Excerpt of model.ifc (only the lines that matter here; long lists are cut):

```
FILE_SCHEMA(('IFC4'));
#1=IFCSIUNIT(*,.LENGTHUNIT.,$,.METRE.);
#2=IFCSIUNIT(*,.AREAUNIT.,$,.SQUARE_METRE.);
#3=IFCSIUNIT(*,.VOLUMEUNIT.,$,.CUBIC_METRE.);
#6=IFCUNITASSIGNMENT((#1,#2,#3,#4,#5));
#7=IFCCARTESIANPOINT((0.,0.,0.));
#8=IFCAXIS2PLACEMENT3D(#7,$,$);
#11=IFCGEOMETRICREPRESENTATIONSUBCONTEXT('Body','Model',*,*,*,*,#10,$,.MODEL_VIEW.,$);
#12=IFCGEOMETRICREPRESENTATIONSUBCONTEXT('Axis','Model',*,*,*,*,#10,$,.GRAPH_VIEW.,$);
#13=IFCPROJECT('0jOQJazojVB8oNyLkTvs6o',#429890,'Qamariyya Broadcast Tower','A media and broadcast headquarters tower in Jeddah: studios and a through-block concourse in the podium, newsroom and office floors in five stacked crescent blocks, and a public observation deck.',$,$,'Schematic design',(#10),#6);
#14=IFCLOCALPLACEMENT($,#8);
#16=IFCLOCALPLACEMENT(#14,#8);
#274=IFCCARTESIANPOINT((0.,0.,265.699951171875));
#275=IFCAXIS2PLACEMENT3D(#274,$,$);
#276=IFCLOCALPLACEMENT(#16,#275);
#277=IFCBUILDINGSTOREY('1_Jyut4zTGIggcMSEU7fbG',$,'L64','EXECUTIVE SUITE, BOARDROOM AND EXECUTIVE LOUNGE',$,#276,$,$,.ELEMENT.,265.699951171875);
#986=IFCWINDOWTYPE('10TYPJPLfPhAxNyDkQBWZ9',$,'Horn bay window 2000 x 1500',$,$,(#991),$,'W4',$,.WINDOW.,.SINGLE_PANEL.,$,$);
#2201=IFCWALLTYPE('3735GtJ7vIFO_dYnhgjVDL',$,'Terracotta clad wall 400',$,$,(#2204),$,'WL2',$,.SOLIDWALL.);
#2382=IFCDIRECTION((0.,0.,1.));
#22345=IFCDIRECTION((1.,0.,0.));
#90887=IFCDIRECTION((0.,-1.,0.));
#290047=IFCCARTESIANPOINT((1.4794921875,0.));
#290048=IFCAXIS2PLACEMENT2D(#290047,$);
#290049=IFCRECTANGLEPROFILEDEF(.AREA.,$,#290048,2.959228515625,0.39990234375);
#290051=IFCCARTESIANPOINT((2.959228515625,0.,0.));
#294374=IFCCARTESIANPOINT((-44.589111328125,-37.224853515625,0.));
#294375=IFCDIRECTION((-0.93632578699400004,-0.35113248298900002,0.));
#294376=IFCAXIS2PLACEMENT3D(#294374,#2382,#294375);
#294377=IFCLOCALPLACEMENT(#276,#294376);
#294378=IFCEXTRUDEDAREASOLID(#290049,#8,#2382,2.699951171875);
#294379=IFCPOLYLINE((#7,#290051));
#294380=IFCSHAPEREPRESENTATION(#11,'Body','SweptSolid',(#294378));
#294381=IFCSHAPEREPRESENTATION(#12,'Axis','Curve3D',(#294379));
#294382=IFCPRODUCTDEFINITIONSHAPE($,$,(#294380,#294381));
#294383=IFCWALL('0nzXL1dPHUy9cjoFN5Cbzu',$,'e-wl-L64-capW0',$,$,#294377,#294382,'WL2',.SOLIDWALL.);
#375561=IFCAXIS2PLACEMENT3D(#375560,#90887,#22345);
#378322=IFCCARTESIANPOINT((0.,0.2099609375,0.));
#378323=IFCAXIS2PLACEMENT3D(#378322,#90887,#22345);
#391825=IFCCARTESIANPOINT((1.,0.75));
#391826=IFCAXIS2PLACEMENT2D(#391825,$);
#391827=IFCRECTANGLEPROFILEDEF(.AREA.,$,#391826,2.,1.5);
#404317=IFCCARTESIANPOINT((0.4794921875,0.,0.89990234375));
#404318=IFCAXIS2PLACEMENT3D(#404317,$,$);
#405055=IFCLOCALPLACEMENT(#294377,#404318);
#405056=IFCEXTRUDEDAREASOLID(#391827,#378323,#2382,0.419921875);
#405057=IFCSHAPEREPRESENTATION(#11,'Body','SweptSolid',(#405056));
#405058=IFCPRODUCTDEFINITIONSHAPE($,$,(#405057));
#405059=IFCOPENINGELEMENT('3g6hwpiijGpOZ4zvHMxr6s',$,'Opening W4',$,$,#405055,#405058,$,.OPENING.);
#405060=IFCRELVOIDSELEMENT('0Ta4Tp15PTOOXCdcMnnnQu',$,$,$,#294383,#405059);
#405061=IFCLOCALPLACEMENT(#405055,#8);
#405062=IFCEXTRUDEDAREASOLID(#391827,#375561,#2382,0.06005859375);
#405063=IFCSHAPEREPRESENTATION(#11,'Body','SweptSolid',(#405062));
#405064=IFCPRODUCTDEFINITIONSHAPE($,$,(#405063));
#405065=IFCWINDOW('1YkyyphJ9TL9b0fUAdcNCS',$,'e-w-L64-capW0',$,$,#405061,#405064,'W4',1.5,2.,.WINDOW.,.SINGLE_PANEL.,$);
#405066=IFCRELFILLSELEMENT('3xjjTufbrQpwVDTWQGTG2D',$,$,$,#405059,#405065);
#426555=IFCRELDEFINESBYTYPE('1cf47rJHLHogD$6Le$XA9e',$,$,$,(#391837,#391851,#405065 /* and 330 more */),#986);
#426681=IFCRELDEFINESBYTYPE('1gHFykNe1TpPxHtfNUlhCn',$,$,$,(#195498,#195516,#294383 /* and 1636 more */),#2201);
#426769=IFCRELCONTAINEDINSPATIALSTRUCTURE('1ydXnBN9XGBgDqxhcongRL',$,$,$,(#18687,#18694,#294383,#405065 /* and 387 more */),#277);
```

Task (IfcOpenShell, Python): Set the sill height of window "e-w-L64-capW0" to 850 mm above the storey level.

```python
import numpy as np
import ifcopenshell
import ifcopenshell.api.geometry
import ifcopenshell.geom
import ifcopenshell.util.element
import ifcopenshell.util.placement
import ifcopenshell.util.shape
import ifcopenshell.util.unit

model = ifcopenshell.open("model.ifc")
unit_scale = ifcopenshell.util.unit.calculate_unit_scale(model)

window = model.by_guid("1YkyyphJ9TL9b0fUAdcNCS")
opening = window.FillsVoids[0].RelatingOpeningElement
storey = ifcopenshell.util.element.get_container(window, ifc_class="IfcBuildingStorey")
level = ifcopenshell.util.placement.get_local_placement(storey.ObjectPlacement)[2, 3]

# The opening's origin need not be at the sill, so measure its lowest point.
shape = ifcopenshell.geom.create_shape(ifcopenshell.geom.settings(), opening)
bottom = ifcopenshell.util.shape.get_shape_bottom_elevation(shape, shape.geometry) / unit_scale
dz = level + 0.85 / unit_scale - bottom

shift = np.array([0.0, 0.0, dz])
# The window is placed relative to its opening, so it follows when the opening moves.
matrix = ifcopenshell.util.placement.get_local_placement(opening.ObjectPlacement)
matrix[:3, 3] += shift
ifcopenshell.api.geometry.edit_object_placement(
    model, product=opening, matrix=matrix, is_si=False, should_transform_children=True
)

print(f"moved by {dz * unit_scale:+.3f} m")

model.write("model_v2.ifc")
```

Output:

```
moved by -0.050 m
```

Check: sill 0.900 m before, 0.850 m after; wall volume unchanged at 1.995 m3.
